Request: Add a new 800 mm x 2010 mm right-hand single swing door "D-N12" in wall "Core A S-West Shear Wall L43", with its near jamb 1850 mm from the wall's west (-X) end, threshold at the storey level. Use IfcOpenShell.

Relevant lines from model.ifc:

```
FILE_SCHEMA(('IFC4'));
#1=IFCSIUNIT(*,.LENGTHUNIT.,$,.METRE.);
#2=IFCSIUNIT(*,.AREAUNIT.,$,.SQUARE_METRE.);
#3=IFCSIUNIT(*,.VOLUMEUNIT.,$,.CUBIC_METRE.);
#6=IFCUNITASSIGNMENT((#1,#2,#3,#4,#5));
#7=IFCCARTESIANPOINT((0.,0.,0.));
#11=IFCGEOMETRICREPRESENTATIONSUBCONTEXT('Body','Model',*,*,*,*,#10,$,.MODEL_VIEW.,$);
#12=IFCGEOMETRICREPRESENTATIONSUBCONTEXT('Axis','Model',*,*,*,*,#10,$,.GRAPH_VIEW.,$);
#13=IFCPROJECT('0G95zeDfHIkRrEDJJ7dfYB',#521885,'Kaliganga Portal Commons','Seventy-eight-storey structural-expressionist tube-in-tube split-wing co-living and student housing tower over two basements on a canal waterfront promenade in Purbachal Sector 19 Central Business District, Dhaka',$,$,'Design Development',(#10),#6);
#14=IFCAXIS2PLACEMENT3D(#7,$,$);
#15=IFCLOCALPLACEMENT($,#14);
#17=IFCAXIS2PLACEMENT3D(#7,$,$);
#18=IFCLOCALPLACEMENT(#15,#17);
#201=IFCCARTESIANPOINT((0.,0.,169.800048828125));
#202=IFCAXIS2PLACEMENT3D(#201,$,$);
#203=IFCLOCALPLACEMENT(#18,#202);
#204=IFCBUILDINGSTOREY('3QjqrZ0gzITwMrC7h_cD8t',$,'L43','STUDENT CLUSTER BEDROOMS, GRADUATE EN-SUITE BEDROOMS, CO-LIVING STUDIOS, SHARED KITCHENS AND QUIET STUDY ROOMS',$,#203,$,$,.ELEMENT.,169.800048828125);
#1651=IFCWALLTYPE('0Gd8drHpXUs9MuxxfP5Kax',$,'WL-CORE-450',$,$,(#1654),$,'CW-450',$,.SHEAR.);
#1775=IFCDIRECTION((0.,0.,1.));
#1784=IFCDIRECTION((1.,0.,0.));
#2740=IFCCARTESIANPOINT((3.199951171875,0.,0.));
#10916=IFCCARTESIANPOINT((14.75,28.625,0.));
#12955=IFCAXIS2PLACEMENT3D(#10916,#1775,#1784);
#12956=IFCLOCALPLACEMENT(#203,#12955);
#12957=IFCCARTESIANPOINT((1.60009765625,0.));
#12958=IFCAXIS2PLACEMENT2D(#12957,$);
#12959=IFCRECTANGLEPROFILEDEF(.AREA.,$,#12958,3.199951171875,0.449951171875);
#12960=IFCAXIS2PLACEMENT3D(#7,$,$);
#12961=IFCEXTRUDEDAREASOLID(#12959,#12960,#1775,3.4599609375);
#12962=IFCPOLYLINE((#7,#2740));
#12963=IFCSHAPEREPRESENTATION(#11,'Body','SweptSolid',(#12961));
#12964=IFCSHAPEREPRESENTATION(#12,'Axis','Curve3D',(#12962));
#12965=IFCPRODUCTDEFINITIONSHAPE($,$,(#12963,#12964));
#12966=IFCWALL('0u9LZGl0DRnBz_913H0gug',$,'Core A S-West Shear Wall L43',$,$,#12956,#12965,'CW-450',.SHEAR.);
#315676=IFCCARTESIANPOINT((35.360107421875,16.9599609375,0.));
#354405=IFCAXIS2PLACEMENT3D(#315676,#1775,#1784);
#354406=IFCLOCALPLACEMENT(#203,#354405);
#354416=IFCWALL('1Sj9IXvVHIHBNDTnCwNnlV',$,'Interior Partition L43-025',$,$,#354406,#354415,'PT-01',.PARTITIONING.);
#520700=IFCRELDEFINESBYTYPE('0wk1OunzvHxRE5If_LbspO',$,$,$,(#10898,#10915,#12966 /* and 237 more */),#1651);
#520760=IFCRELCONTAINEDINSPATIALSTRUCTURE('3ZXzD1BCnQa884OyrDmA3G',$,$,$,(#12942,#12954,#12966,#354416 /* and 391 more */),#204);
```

```python
import numpy as np
import ifcopenshell
import ifcopenshell.api.feature
import ifcopenshell.api.geometry
import ifcopenshell.api.root
import ifcopenshell.api.spatial
import ifcopenshell.geom
import ifcopenshell.util.element
import ifcopenshell.util.placement
import ifcopenshell.util.representation
import ifcopenshell.util.shape
import ifcopenshell.util.unit

model = ifcopenshell.open("model.ifc")
unit_scale = ifcopenshell.util.unit.calculate_unit_scale(model)
settings = ifcopenshell.geom.settings()


def volume(element):
    """Net volume in cubic metres, openings subtracted."""
    shape = ifcopenshell.geom.create_shape(settings, element)
    return ifcopenshell.util.shape.get_volume(shape.geometry)


wall = model.by_guid("0u9LZGl0DRnBz_913H0gug")
storey = ifcopenshell.util.element.get_container(wall, ifc_class="IfcBuildingStorey")
context = ifcopenshell.util.representation.get_context(model, "Model", "Body", "MODEL_VIEW")
before = volume(wall)

width, height, from_end, sill = 0.8, 2.01, 1.85, 0.0  # metres

# The wall runs along its own X axis, and the end named is its -X end.
wall_shape = ifcopenshell.geom.create_shape(settings, wall)
x, y, z = ifcopenshell.util.shape.get_vertices(wall_shape.geometry).T
start = x.min() + from_end
face, thickness = float(y.min()), float(y.max() - y.min())
wall_matrix = ifcopenshell.util.placement.get_local_placement(wall.ObjectPlacement)
level = ifcopenshell.util.placement.get_local_placement(storey.ObjectPlacement)[2, 3]


def in_wall(x, y):
    """Placement at x, y metres in the wall's axes, at sill height."""
    matrix = wall_matrix.copy()
    matrix[:, 3] = wall_matrix @ np.array([x / unit_scale, y / unit_scale, 0.0, 1.0])
    matrix[2, 3] = level + sill / unit_scale
    return matrix


# Opening: a box that overshoots both wall faces by 50 mm.
opening = ifcopenshell.api.root.create_entity(model, ifc_class="IfcOpeningElement", predefined_type="OPENING")
box = ifcopenshell.api.geometry.add_wall_representation(
    model, context=context, length=width, height=height, thickness=thickness + 0.1
)
ifcopenshell.api.geometry.assign_representation(model, product=opening, representation=box)
ifcopenshell.api.geometry.edit_object_placement(model, product=opening, matrix=in_wall(start, face - 0.05), is_si=False)
ifcopenshell.api.feature.add_feature(model, feature=opening, element=wall)

door = ifcopenshell.api.root.create_entity(model, ifc_class="IfcDoor", name="D-N12", predefined_type="DOOR")
door.OverallWidth, door.OverallHeight = width / unit_scale, height / unit_scale
door.OperationType = "SINGLE_SWING_RIGHT"
body = ifcopenshell.api.geometry.add_door_representation(
    model,
    context=context,
    overall_width=door.OverallWidth,
    overall_height=door.OverallHeight,
    operation_type="SINGLE_SWING_RIGHT",
    lining_properties={"LiningDepth": thickness / unit_scale, "ThresholdDepth": thickness / unit_scale},
)
ifcopenshell.api.geometry.assign_representation(model, product=door, representation=body)
ifcopenshell.api.spatial.assign_container(model, products=[door], relating_structure=storey)
ifcopenshell.api.feature.add_filling(model, opening=opening, element=door)

# The lining spans the wall, so the door starts at the wall face.
ifcopenshell.api.geometry.edit_object_placement(model, product=door, matrix=in_wall(start, face), is_si=False)

after = volume(wall)

print(f"wall volume {before:.3f} -> {after:.3f} m3")

model.write("model_rev.ifc")
```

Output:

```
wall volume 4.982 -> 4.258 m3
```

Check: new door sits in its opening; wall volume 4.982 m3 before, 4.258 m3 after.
